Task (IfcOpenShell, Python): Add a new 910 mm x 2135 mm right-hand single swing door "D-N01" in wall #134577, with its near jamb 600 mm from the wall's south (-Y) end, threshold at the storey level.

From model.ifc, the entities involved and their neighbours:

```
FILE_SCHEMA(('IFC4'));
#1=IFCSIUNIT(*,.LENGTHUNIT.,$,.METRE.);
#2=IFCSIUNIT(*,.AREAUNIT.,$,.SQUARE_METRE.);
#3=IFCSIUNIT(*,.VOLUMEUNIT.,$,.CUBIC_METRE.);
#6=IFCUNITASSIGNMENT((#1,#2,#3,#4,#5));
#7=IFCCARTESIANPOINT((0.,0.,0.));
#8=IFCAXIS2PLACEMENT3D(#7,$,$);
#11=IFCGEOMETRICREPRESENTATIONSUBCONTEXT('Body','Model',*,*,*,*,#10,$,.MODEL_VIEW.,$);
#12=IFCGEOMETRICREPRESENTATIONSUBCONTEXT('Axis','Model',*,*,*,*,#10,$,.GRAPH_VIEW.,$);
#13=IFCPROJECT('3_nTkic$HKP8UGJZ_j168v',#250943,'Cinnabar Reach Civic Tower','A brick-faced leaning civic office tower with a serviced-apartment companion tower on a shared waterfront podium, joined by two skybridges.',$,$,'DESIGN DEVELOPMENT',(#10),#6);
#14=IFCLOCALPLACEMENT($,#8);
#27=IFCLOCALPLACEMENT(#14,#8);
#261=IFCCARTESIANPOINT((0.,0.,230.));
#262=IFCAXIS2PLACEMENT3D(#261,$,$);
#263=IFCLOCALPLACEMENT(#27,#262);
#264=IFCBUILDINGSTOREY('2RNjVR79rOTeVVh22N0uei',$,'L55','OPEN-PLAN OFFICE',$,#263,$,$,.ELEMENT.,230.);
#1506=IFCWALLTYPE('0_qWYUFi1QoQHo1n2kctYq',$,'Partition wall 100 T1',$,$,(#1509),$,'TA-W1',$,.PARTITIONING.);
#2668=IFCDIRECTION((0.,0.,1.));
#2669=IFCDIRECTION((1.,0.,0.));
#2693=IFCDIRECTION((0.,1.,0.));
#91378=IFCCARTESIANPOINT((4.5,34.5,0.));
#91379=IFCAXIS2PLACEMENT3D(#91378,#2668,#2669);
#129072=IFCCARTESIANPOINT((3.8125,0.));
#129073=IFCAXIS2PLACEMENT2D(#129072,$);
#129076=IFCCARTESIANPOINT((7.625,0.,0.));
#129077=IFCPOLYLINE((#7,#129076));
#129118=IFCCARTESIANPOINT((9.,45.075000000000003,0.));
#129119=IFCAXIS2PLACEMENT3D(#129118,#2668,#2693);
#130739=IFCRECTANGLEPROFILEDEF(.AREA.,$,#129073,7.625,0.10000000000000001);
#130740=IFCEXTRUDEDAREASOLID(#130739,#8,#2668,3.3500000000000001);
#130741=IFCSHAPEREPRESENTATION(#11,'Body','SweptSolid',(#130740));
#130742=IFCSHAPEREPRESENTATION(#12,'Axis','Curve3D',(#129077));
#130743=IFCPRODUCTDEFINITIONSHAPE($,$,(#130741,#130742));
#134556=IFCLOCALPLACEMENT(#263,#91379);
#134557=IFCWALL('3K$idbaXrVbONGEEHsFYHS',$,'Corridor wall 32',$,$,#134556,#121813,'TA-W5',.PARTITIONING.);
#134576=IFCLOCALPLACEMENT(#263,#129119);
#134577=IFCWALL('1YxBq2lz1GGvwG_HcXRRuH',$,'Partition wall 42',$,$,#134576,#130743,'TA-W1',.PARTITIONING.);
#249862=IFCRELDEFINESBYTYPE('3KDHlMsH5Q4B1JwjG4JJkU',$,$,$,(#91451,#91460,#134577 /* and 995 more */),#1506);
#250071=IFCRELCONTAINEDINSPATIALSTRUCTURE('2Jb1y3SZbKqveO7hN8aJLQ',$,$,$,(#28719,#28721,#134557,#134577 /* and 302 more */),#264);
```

```python
import numpy as np
import ifcopenshell
import ifcopenshell.api.feature
import ifcopenshell.api.geometry
import ifcopenshell.api.root
import ifcopenshell.api.spatial
import ifcopenshell.geom
import ifcopenshell.util.element
import ifcopenshell.util.placement
import ifcopenshell.util.representation
import ifcopenshell.util.shape
import ifcopenshell.util.unit

model = ifcopenshell.open("model.ifc")
unit_scale = ifcopenshell.util.unit.calculate_unit_scale(model)
settings = ifcopenshell.geom.settings()


def volume(element):
    """Net volume in cubic metres, openings subtracted."""
    shape = ifcopenshell.geom.create_shape(settings, element)
    return ifcopenshell.util.shape.get_volume(shape.geometry)


wall = model.by_guid("1YxBq2lz1GGvwG_HcXRRuH")
storey = ifcopenshell.util.element.get_container(wall, ifc_class="IfcBuildingStorey")
context = ifcopenshell.util.representation.get_context(model, "Model", "Body", "MODEL_VIEW")
before = volume(wall)

width, height, from_end, sill = 0.91, 2.135, 0.6, 0.0  # metres

# The wall runs along its own X axis, and the end named is its -X end.
wall_shape = ifcopenshell.geom.create_shape(settings, wall)
x, y, z = ifcopenshell.util.shape.get_vertices(wall_shape.geometry).T
start = x.min() + from_end
face, thickness = float(y.min()), float(y.max() - y.min())
wall_matrix = ifcopenshell.util.placement.get_local_placement(wall.ObjectPlacement)
level = ifcopenshell.util.placement.get_local_placement(storey.ObjectPlacement)[2, 3]


def in_wall(x, y):
    """Placement at x, y metres in the wall's axes, at sill height."""
    matrix = wall_matrix.copy()
    matrix[:, 3] = wall_matrix @ np.array([x / unit_scale, y / unit_scale, 0.0, 1.0])
    matrix[2, 3] = level + sill / unit_scale
    return matrix


# Opening: a box that overshoots both wall faces by 50 mm.
opening = ifcopenshell.api.root.create_entity(model, ifc_class="IfcOpeningElement", predefined_type="OPENING")
box = ifcopenshell.api.geometry.add_wall_representation(
    model, context=context, length=width, height=height, thickness=thickness + 0.1
)
ifcopenshell.api.geometry.assign_representation(model, product=opening, representation=box)
ifcopenshell.api.geometry.edit_object_placement(model, product=opening, matrix=in_wall(start, face - 0.05), is_si=False)
ifcopenshell.api.feature.add_feature(model, feature=opening, element=wall)

door = ifcopenshell.api.root.create_entity(model, ifc_class="IfcDoor", name="D-N01", predefined_type="DOOR")
door.OverallWidth, door.OverallHeight = width / unit_scale, height / unit_scale
door.OperationType = "SINGLE_SWING_RIGHT"
body = ifcopenshell.api.geometry.add_door_representation(
    model,
    context=context,
    overall_width=door.OverallWidth,
    overall_height=door.OverallHeight,
    operation_type="SINGLE_SWING_RIGHT",
    lining_properties={"LiningDepth": thickness / unit_scale, "ThresholdDepth": thickness / unit_scale},
)
ifcopenshell.api.geometry.assign_representation(model, product=door, representation=body)
ifcopenshell.api.spatial.assign_container(model, products=[door], relating_structure=storey)
ifcopenshell.api.feature.add_filling(model, opening=opening, element=door)

# The lining spans the wall, so the door starts at the wall face.
ifcopenshell.api.geometry.edit_object_placement(model, product=door, matrix=in_wall(start, face), is_si=False)

after = volume(wall)

print(f"wall volume {before:.3f} -> {after:.3f} m3")

model.write("model_edited.ifc")
```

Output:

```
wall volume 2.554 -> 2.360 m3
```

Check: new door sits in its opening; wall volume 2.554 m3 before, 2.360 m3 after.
